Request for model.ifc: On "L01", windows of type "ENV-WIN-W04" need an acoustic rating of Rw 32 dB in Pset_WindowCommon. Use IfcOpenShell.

First a look at what the model holds.

```python
import ifcopenshell
import ifcopenshell.util.element

model = ifcopenshell.open("model.ifc")
print(model.schema)
storey = next(s for s in model.by_type("IfcBuildingStorey") if s.Name == "L01")
windows = [e for e in ifcopenshell.util.element.get_decomposition(storey) if e.is_a("IfcWindow")]
seen = {}
for e in windows:
    element_type = ifcopenshell.util.element.get_type(e)
    key = (element_type.Name if element_type != e and element_type else None, ifcopenshell.util.element.get_pset(e, "Pset_WindowCommon", "AcousticRating"))
    seen[key] = seen.get(key, 0) + 1
for (name, value), count in sorted(seen.items(), key=str):
    print(count, "x", name, "|", value)
```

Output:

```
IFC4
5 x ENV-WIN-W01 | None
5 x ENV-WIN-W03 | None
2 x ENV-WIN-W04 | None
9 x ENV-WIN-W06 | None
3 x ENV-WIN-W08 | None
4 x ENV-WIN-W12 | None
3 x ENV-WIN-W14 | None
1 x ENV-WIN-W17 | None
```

```python
import ifcopenshell
import ifcopenshell.api.pset
import ifcopenshell.util.element

model = ifcopenshell.open("model.ifc")

storey = next(s for s in model.by_type("IfcBuildingStorey") if s.Name == "L01")
windows = [e for e in ifcopenshell.util.element.get_decomposition(storey) if e.is_a("IfcWindow")]

count = 0
for e in windows:
    element_type = ifcopenshell.util.element.get_type(e)
    if element_type in (None, e) or element_type.Name != "ENV-WIN-W04":
        continue
    # add_pset returns the element's existing set when there is one.
    pset = ifcopenshell.api.pset.add_pset(model, product=e, name="Pset_WindowCommon")
    ifcopenshell.api.pset.edit_pset(model, pset=pset, properties={"AcousticRating": "Rw 32 dB"})
    count += 1

print(count, "windows updated")

model.write("model-out.ifc")
```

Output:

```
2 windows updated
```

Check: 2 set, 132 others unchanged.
